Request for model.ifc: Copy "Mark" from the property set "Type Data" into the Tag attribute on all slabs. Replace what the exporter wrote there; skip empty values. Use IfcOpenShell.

First a look at what the model holds.

```python
import ifcopenshell
import ifcopenshell.util.element

model = ifcopenshell.open("model.ifc")
print(model.schema)
slabs = model.by_type("IfcSlab")
print(len(slabs), "slabs")
for e in slabs[:8]:
    source = ifcopenshell.util.element.get_pset(e, "Type Data", "Mark")
    target = e.Tag
    print(e.id(), repr(source), repr(target), sep=" | ")
```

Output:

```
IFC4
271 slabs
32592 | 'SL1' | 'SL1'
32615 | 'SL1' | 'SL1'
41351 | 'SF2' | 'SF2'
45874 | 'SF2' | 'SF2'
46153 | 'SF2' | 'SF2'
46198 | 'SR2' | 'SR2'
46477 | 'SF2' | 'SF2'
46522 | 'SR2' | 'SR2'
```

```python
import ifcopenshell
import ifcopenshell.util.element

model = ifcopenshell.open("model.ifc")

count = 0
for e in model.by_type("IfcSlab"):
    value = ifcopenshell.util.element.get_pset(e, "Type Data", "Mark")
    current = e.Tag
    if not value or not value.strip() or current == value:
        continue
    e.Tag = value
    count += 1

print(count, "slabs updated")

model.write("model_edited.ifc")
```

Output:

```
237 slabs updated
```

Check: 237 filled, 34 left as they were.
